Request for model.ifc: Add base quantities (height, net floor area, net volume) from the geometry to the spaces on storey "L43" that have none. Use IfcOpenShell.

First a look at what the model holds.

```python
import ifcopenshell
import ifcopenshell.util.element
import ifcopenshell.util.unit

model = ifcopenshell.open("model.ifc")
print(model.schema)
for unit_type in ("LENGTHUNIT", "AREAUNIT", "VOLUMEUNIT"):
    print(unit_type, ifcopenshell.util.unit.calculate_unit_scale(model, unit_type))
storey = next(s for s in model.by_type("IfcBuildingStorey") if s.Name == "L43")
spaces = [e for e in ifcopenshell.util.element.get_decomposition(storey) if e.is_a("IfcSpace")]
for e in sorted(spaces, key=lambda e: e.id()):
    print(e.id(), e.is_a(), e.Name, list(ifcopenshell.util.element.get_psets(e, qtos_only=True)), sep=" | ")
```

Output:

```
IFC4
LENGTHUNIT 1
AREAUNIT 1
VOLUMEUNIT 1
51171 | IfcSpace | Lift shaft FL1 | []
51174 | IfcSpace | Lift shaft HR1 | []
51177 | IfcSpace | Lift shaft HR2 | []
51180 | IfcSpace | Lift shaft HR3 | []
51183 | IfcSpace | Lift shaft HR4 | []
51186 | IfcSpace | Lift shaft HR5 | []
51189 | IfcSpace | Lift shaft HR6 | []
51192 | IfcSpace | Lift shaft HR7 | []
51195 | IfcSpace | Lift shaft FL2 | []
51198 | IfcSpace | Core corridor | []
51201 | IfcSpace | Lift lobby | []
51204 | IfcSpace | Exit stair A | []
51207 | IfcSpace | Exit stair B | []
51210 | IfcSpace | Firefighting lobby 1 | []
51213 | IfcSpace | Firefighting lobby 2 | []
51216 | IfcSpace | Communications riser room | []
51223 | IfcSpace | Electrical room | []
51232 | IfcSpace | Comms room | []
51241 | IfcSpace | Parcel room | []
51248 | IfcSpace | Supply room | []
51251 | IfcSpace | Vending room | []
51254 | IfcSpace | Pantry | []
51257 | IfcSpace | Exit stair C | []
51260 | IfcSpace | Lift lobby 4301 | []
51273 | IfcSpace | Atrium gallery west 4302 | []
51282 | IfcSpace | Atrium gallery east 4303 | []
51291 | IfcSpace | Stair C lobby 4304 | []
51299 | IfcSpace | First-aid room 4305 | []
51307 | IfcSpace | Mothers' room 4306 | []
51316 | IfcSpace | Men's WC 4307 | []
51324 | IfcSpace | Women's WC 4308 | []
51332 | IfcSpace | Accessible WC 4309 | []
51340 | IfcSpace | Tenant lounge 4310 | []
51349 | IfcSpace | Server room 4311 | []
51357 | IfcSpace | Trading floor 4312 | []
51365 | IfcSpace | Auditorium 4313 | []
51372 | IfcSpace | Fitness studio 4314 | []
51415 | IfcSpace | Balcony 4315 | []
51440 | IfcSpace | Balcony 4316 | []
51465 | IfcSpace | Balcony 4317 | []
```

```python
import ifcopenshell
import ifcopenshell.api.pset
import ifcopenshell.geom
import ifcopenshell.util.element
import ifcopenshell.util.shape
import ifcopenshell.util.unit

model = ifcopenshell.open("model.ifc")
unit_scale = ifcopenshell.util.unit.calculate_unit_scale(model)
area_scale = ifcopenshell.util.unit.calculate_unit_scale(model, "AREAUNIT")
volume_scale = ifcopenshell.util.unit.calculate_unit_scale(model, "VOLUMEUNIT")
settings = ifcopenshell.geom.settings()

storey = next(s for s in model.by_type("IfcBuildingStorey") if s.Name == "L43")
spaces = [e for e in ifcopenshell.util.element.get_decomposition(storey) if e.is_a("IfcSpace")]

for e in sorted(spaces, key=lambda e: e.id()):
    if ifcopenshell.util.element.get_psets(e, qtos_only=True, should_inherit=False):
        continue
    # Geometry comes back in metres, in the element's own axes.
    shape = ifcopenshell.geom.create_shape(settings, e)
    values = {
        "Height": ifcopenshell.util.shape.get_z(shape.geometry) / unit_scale,
        "NetFloorArea": ifcopenshell.util.shape.get_footprint_area(shape.geometry) / area_scale,
        "NetVolume": ifcopenshell.util.shape.get_volume(shape.geometry) / volume_scale,
    }
    qto = ifcopenshell.api.pset.add_qto(model, product=e, name="Qto_SpaceBaseQuantities")
    ifcopenshell.api.pset.edit_qto(model, qto=qto, properties=values)
    print(e.id(), {k: round(v, 3) for k, v in values.items()})

model.write("model_rev.ifc")
```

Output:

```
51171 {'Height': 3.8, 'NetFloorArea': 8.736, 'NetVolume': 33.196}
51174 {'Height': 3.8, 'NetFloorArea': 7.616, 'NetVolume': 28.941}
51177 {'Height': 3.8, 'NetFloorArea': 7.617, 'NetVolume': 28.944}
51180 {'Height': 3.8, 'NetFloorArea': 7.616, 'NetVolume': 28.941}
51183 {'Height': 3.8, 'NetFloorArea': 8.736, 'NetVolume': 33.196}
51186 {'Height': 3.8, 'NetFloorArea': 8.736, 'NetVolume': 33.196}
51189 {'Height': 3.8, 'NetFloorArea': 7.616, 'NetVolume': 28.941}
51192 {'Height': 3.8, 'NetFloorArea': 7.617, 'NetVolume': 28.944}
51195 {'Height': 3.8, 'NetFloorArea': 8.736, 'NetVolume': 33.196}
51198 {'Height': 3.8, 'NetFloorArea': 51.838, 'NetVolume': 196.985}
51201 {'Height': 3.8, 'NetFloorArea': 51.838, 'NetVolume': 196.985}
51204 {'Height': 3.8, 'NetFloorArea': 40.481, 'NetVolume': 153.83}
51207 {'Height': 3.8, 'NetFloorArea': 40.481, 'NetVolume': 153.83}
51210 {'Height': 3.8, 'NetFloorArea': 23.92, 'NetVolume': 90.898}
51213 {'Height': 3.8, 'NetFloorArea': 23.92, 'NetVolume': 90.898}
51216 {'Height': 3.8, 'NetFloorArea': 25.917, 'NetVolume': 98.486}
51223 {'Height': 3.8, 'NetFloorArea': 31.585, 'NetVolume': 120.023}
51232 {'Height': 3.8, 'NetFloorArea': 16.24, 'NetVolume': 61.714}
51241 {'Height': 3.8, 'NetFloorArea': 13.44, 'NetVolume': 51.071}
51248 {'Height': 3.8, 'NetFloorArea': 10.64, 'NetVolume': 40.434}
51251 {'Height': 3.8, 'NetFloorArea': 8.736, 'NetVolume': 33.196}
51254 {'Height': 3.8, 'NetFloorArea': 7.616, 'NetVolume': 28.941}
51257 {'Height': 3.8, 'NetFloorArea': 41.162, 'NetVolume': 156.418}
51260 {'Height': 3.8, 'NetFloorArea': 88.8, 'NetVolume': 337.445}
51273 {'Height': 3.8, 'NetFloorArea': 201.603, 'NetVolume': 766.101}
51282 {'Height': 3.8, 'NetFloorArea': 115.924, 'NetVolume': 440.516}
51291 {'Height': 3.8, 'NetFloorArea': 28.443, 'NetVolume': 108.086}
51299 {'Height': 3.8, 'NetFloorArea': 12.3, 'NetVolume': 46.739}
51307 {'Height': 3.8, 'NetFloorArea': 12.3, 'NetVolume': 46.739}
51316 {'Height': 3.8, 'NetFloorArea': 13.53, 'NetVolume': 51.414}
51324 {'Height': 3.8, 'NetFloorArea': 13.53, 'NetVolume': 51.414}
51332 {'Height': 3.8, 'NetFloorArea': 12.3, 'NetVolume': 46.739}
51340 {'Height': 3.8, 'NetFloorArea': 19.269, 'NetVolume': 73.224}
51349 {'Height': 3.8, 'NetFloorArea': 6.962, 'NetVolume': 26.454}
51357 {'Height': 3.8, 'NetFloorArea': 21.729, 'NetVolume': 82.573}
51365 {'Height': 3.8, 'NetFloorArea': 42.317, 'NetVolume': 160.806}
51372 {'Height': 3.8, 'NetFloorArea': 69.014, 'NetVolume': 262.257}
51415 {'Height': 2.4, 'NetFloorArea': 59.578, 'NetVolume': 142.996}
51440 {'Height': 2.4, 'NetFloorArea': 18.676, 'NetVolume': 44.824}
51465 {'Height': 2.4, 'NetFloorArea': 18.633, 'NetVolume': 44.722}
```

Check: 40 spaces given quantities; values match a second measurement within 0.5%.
